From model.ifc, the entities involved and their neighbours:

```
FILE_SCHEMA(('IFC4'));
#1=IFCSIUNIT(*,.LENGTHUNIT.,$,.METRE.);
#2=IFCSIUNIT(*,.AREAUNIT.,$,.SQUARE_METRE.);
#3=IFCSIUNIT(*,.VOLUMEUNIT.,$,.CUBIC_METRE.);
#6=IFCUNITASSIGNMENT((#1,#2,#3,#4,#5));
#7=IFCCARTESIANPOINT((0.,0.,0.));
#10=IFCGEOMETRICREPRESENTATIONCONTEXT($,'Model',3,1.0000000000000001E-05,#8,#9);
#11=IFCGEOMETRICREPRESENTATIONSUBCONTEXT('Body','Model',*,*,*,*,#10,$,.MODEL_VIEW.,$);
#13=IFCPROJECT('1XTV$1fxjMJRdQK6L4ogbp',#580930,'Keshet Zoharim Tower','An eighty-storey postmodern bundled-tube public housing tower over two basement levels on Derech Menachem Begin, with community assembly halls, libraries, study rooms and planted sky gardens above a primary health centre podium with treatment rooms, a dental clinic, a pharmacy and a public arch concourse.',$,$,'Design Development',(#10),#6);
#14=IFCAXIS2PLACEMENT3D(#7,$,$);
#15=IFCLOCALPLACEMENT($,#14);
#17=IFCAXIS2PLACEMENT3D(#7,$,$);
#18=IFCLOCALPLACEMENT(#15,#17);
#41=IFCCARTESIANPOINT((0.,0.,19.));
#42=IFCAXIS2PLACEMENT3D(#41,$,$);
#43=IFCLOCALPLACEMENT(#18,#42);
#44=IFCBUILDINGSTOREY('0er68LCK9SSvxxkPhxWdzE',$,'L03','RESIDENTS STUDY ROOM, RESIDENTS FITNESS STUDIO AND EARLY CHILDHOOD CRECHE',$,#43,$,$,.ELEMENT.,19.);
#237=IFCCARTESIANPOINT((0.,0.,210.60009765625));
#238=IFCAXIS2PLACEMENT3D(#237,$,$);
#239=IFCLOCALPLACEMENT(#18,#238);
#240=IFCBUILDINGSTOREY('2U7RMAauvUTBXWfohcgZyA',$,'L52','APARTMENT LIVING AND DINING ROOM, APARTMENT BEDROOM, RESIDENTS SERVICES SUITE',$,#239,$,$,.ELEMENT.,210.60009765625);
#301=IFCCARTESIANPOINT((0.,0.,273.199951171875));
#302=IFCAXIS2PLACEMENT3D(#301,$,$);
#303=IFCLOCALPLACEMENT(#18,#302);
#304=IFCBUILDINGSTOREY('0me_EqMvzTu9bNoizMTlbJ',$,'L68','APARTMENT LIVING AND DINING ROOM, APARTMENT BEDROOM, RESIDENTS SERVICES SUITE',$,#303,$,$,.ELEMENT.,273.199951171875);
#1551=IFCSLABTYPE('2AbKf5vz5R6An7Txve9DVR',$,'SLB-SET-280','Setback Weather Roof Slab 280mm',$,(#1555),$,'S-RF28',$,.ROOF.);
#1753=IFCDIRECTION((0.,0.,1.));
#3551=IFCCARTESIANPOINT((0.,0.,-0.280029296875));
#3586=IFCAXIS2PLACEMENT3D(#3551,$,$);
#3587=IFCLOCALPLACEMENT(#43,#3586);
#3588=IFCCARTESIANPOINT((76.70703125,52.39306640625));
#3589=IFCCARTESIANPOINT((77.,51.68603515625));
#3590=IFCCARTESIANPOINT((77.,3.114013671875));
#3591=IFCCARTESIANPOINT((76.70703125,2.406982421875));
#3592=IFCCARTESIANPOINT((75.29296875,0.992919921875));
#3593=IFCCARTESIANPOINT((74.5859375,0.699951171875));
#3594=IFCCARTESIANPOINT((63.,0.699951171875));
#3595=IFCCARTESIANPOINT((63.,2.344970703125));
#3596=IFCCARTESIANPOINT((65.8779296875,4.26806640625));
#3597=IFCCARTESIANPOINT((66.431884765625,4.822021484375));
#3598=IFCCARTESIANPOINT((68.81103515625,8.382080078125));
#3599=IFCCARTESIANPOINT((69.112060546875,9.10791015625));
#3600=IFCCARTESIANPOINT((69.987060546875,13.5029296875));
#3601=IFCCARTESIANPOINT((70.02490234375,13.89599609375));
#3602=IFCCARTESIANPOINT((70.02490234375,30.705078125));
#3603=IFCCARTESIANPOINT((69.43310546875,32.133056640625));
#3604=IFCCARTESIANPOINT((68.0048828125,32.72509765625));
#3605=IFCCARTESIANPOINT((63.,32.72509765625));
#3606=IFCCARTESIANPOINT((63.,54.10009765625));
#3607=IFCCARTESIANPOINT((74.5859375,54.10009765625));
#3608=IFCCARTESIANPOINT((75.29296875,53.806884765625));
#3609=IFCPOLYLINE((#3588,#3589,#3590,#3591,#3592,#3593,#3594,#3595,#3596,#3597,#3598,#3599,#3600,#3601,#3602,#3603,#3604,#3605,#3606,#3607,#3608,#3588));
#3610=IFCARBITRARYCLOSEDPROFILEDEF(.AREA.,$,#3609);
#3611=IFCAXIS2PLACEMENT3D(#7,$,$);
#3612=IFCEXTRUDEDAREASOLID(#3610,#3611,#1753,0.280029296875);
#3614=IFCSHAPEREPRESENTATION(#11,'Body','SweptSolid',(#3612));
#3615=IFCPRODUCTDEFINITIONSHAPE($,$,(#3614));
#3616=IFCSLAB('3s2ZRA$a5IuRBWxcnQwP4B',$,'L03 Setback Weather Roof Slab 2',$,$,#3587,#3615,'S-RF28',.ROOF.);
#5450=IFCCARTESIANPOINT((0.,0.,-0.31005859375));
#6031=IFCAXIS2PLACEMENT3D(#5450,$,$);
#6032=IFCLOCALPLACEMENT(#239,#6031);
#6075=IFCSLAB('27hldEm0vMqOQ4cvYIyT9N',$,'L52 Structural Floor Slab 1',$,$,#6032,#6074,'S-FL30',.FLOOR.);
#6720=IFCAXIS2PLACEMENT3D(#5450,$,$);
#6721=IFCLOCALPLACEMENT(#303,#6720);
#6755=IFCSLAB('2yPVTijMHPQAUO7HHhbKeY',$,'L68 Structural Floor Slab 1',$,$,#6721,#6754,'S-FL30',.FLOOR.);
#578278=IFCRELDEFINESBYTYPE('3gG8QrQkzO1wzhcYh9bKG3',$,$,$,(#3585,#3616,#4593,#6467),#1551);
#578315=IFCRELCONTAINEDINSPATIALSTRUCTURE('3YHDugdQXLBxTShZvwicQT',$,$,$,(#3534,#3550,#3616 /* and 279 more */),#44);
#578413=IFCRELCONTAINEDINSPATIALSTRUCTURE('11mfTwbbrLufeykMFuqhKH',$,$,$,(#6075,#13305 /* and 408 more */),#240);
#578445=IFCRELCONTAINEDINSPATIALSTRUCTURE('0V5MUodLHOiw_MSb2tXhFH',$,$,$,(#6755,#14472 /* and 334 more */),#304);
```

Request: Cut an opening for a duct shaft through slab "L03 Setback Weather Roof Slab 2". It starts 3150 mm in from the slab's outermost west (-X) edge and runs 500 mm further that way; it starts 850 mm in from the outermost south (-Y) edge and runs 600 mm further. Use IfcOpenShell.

```python
import numpy as np
import ifcopenshell
import ifcopenshell.api.feature
import ifcopenshell.api.geometry
import ifcopenshell.api.root
import ifcopenshell.geom
import ifcopenshell.util.placement
import ifcopenshell.util.representation
import ifcopenshell.util.shape
import ifcopenshell.util.unit

model = ifcopenshell.open("model.ifc")
unit_scale = ifcopenshell.util.unit.calculate_unit_scale(model)
settings = ifcopenshell.geom.settings()


def volume(element):
    """Net volume in cubic metres, openings subtracted."""
    shape = ifcopenshell.geom.create_shape(settings, element)
    return ifcopenshell.util.shape.get_volume(shape.geometry)


slab = model.by_guid("3s2ZRA$a5IuRBWxcnQwP4B")
before = volume(slab)

# Extent in the slab's own axes, in metres. The edges named are its -X and -Y sides.
slab_shape = ifcopenshell.geom.create_shape(settings, slab)
vertices = ifcopenshell.util.shape.get_vertices(slab_shape.geometry)
x_min, y_min, bottom = vertices.min(axis=0)
top = vertices[:, 2].max()

opening = ifcopenshell.api.root.create_entity(model, ifc_class="IfcOpeningElement", name="Duct shaft opening", predefined_type="OPENING")
context = ifcopenshell.util.representation.get_context(model, "Model", "Body", "MODEL_VIEW")
width, depth = 0.5, 0.6
outline = [(0.0, 0.0), (width, 0.0), (width, depth), (0.0, depth), (0.0, 0.0)]
# Overshoot both faces by 50 mm so the cut is clean.
shape = ifcopenshell.api.geometry.add_slab_representation(
    model, context=context, depth=top - bottom + 0.1, polyline=outline
)
ifcopenshell.api.geometry.assign_representation(model, product=opening, representation=shape)

matrix = ifcopenshell.util.placement.get_local_placement(slab.ObjectPlacement)
matrix[:, 3] = matrix @ np.append(np.array([x_min + 3.15, y_min + 0.85, bottom - 0.05]) / unit_scale, 1.0)
ifcopenshell.api.geometry.edit_object_placement(model, product=opening, matrix=matrix, is_si=False)
ifcopenshell.api.feature.add_feature(model, feature=opening, element=slab)

after = volume(slab)

print(f"slab volume {before:.3f} -> {after:.3f} m3")

model.write("model-out.ifc")
```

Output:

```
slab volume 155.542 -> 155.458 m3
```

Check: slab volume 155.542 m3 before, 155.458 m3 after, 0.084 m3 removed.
